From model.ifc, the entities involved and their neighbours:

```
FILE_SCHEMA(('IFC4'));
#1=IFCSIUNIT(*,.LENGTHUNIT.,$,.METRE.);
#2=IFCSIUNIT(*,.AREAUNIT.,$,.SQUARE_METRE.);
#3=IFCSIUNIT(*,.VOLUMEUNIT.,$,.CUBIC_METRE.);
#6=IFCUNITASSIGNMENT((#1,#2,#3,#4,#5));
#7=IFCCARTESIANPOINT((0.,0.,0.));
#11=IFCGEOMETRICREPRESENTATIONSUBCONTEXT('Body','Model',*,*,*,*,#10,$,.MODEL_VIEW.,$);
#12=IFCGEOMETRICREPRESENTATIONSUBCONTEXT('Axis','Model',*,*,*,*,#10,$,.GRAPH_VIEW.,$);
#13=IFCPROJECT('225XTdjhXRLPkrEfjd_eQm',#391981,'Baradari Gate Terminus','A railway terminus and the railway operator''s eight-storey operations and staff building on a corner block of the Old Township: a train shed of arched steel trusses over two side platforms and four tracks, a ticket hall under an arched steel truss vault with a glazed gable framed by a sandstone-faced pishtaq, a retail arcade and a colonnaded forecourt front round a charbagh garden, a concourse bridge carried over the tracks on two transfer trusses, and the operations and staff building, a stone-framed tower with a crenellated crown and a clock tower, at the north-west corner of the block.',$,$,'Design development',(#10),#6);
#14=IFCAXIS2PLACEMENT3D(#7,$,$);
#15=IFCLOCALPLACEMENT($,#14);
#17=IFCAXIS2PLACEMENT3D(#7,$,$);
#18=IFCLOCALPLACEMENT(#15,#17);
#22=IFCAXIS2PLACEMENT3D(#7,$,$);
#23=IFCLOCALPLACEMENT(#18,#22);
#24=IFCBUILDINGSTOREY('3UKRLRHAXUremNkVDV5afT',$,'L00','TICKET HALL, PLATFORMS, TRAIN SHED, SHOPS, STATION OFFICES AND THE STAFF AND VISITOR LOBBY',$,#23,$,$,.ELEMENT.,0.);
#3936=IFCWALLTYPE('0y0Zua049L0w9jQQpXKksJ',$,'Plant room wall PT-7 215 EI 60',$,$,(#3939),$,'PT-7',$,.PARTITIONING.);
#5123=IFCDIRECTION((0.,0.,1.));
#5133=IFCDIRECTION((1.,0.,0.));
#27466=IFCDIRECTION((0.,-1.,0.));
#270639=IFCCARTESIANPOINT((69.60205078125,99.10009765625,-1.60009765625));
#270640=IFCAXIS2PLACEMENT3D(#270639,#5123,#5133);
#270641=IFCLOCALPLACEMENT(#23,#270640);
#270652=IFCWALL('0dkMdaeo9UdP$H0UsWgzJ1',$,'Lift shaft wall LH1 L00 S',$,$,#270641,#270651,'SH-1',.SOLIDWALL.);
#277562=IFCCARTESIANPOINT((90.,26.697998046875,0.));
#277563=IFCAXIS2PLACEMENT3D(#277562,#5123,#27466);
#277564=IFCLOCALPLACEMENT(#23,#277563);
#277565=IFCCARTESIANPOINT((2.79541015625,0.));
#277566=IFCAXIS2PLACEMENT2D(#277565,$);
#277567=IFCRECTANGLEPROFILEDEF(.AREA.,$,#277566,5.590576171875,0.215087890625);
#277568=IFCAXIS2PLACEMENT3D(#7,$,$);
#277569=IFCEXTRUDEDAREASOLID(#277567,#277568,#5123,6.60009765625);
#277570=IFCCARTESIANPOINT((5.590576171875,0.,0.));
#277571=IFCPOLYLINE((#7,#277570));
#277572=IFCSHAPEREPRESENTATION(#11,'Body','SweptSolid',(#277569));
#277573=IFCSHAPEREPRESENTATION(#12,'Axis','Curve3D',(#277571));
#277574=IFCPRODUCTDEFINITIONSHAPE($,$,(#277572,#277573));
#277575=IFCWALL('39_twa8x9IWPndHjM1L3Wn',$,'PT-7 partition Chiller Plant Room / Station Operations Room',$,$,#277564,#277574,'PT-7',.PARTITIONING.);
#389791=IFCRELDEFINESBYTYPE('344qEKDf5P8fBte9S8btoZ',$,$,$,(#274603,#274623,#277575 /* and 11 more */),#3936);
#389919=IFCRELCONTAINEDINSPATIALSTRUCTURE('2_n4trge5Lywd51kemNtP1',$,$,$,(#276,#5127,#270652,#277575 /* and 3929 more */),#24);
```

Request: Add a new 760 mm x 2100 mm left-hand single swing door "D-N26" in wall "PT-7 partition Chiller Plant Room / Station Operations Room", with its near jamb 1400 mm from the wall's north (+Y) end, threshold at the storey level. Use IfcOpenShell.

```python
import numpy as np
import ifcopenshell
import ifcopenshell.api.feature
import ifcopenshell.api.geometry
import ifcopenshell.api.root
import ifcopenshell.api.spatial
import ifcopenshell.geom
import ifcopenshell.util.element
import ifcopenshell.util.placement
import ifcopenshell.util.representation
import ifcopenshell.util.shape
import ifcopenshell.util.unit

model = ifcopenshell.open("model.ifc")
unit_scale = ifcopenshell.util.unit.calculate_unit_scale(model)
settings = ifcopenshell.geom.settings()


def volume(element):
    """Net volume in cubic metres, openings subtracted."""
    shape = ifcopenshell.geom.create_shape(settings, element)
    return ifcopenshell.util.shape.get_volume(shape.geometry)


wall = model.by_guid("39_twa8x9IWPndHjM1L3Wn")
storey = ifcopenshell.util.element.get_container(wall, ifc_class="IfcBuildingStorey")
context = ifcopenshell.util.representation.get_context(model, "Model", "Body", "MODEL_VIEW")
before = volume(wall)

width, height, from_end, sill = 0.76, 2.1, 1.4, 0.0  # metres

# The wall runs along its own X axis, and the end named is its -X end.
wall_shape = ifcopenshell.geom.create_shape(settings, wall)
x, y, z = ifcopenshell.util.shape.get_vertices(wall_shape.geometry).T
start = x.min() + from_end
face, thickness = float(y.min()), float(y.max() - y.min())
wall_matrix = ifcopenshell.util.placement.get_local_placement(wall.ObjectPlacement)
level = ifcopenshell.util.placement.get_local_placement(storey.ObjectPlacement)[2, 3]


def in_wall(x, y):
    """Placement at x, y metres in the wall's axes, at sill height."""
    matrix = wall_matrix.copy()
    matrix[:, 3] = wall_matrix @ np.array([x / unit_scale, y / unit_scale, 0.0, 1.0])
    matrix[2, 3] = level + sill / unit_scale
    return matrix


# Opening: a box that overshoots both wall faces by 50 mm.
opening = ifcopenshell.api.root.create_entity(model, ifc_class="IfcOpeningElement", predefined_type="OPENING")
box = ifcopenshell.api.geometry.add_wall_representation(
    model, context=context, length=width, height=height, thickness=thickness + 0.1
)
ifcopenshell.api.geometry.assign_representation(model, product=opening, representation=box)
ifcopenshell.api.geometry.edit_object_placement(model, product=opening, matrix=in_wall(start, face - 0.05), is_si=False)
ifcopenshell.api.feature.add_feature(model, feature=opening, element=wall)

door = ifcopenshell.api.root.create_entity(model, ifc_class="IfcDoor", name="D-N26", predefined_type="DOOR")
door.OverallWidth, door.OverallHeight = width / unit_scale, height / unit_scale
door.OperationType = "SINGLE_SWING_LEFT"
body = ifcopenshell.api.geometry.add_door_representation(
    model,
    context=context,
    overall_width=door.OverallWidth,
    overall_height=door.OverallHeight,
    operation_type="SINGLE_SWING_LEFT",
    lining_properties={"LiningDepth": thickness / unit_scale, "ThresholdDepth": thickness / unit_scale},
)
ifcopenshell.api.geometry.assign_representation(model, product=door, representation=body)
ifcopenshell.api.spatial.assign_container(model, products=[door], relating_structure=storey)
ifcopenshell.api.feature.add_filling(model, opening=opening, element=door)

# The lining spans the wall, so the door starts at the wall face.
ifcopenshell.api.geometry.edit_object_placement(model, product=door, matrix=in_wall(start, face), is_si=False)

after = volume(wall)

print(f"wall volume {before:.3f} -> {after:.3f} m3")

model.write("model_rev.ifc")
```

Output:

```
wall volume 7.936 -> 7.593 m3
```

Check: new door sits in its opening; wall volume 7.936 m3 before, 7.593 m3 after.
